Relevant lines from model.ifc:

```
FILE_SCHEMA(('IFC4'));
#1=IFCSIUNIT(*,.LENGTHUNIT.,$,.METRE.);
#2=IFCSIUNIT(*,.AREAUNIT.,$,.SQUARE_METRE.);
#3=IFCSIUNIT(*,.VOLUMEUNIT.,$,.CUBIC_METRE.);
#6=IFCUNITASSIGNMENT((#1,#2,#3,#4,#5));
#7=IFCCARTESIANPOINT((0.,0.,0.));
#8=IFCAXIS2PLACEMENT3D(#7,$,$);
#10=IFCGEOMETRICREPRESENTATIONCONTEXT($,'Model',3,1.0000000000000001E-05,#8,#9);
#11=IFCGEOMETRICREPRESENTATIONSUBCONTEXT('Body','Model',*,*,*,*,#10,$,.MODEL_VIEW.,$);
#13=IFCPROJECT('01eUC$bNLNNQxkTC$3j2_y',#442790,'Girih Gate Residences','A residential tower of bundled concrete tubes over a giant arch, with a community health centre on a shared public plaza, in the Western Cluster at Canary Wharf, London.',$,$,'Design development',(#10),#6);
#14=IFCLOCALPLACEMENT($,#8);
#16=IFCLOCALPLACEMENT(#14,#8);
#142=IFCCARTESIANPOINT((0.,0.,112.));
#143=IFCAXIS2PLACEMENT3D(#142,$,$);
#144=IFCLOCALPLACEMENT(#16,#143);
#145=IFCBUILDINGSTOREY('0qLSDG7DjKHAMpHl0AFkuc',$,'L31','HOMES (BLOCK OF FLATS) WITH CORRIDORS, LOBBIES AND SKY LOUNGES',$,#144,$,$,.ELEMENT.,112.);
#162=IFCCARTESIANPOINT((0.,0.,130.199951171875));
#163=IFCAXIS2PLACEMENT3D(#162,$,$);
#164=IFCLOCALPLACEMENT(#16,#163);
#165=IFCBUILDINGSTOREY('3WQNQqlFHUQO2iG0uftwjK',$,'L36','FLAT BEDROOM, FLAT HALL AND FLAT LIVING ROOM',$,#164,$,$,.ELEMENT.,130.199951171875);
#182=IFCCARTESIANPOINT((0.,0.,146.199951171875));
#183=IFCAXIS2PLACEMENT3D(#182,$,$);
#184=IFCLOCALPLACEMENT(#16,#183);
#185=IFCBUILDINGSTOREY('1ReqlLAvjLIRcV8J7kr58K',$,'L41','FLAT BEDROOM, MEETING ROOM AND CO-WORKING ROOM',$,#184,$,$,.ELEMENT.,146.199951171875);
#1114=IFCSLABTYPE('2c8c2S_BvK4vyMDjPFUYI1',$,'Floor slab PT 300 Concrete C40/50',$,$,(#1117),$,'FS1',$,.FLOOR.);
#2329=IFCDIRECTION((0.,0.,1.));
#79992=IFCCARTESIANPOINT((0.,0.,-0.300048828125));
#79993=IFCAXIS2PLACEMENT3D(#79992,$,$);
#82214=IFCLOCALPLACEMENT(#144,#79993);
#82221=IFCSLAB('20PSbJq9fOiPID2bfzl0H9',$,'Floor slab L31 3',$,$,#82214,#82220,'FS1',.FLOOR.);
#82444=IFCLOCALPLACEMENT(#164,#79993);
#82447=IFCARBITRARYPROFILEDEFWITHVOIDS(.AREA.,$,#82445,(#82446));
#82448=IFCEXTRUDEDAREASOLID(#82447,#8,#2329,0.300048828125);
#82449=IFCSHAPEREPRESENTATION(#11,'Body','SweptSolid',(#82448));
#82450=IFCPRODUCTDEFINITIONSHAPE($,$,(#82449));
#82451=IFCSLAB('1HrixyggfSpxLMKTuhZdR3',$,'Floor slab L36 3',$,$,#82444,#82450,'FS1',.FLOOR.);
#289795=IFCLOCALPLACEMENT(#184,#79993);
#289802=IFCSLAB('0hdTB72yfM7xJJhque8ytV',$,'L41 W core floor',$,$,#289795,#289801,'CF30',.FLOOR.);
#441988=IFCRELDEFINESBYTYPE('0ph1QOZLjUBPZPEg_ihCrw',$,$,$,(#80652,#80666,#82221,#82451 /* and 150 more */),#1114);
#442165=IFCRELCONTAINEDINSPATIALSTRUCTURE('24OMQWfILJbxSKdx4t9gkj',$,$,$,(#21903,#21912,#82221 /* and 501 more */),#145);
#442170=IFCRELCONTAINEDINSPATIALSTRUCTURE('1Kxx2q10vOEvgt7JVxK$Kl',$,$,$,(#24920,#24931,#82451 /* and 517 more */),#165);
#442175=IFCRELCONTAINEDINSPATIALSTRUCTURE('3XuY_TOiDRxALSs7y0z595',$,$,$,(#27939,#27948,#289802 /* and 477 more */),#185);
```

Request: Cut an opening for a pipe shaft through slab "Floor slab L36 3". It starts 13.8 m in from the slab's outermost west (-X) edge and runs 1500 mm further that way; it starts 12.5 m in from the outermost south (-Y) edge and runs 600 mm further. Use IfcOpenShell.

```python
import numpy as np
import ifcopenshell
import ifcopenshell.api.feature
import ifcopenshell.api.geometry
import ifcopenshell.api.root
import ifcopenshell.geom
import ifcopenshell.util.placement
import ifcopenshell.util.representation
import ifcopenshell.util.shape
import ifcopenshell.util.unit

model = ifcopenshell.open("model.ifc")
unit_scale = ifcopenshell.util.unit.calculate_unit_scale(model)
settings = ifcopenshell.geom.settings()


def volume(element):
    """Net volume in cubic metres, openings subtracted."""
    shape = ifcopenshell.geom.create_shape(settings, element)
    return ifcopenshell.util.shape.get_volume(shape.geometry)


slab = model.by_id(82451)
before = volume(slab)

# Extent in the slab's own axes, in metres. The edges named are its -X and -Y sides.
slab_shape = ifcopenshell.geom.create_shape(settings, slab)
vertices = ifcopenshell.util.shape.get_vertices(slab_shape.geometry)
x_min, y_min, bottom = vertices.min(axis=0)
top = vertices[:, 2].max()

opening = ifcopenshell.api.root.create_entity(model, ifc_class="IfcOpeningElement", name="Pipe shaft opening", predefined_type="OPENING")
context = ifcopenshell.util.representation.get_context(model, "Model", "Body", "MODEL_VIEW")
width, depth = 1.5, 0.6
outline = [(0.0, 0.0), (width, 0.0), (width, depth), (0.0, depth), (0.0, 0.0)]
# Overshoot both faces by 50 mm so the cut is clean.
shape = ifcopenshell.api.geometry.add_slab_representation(
    model, context=context, depth=top - bottom + 0.1, polyline=outline
)
ifcopenshell.api.geometry.assign_representation(model, product=opening, representation=shape)

matrix = ifcopenshell.util.placement.get_local_placement(slab.ObjectPlacement)
matrix[:, 3] = matrix @ np.append(np.array([x_min + 13.8, y_min + 12.5, bottom - 0.05]) / unit_scale, 1.0)
ifcopenshell.api.geometry.edit_object_placement(model, product=opening, matrix=matrix, is_si=False)
ifcopenshell.api.feature.add_feature(model, feature=opening, element=slab)

after = volume(slab)

print(f"slab volume {before:.3f} -> {after:.3f} m3")

model.write("model_v2.ifc")
```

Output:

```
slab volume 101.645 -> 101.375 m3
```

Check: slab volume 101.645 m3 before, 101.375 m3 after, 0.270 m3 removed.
